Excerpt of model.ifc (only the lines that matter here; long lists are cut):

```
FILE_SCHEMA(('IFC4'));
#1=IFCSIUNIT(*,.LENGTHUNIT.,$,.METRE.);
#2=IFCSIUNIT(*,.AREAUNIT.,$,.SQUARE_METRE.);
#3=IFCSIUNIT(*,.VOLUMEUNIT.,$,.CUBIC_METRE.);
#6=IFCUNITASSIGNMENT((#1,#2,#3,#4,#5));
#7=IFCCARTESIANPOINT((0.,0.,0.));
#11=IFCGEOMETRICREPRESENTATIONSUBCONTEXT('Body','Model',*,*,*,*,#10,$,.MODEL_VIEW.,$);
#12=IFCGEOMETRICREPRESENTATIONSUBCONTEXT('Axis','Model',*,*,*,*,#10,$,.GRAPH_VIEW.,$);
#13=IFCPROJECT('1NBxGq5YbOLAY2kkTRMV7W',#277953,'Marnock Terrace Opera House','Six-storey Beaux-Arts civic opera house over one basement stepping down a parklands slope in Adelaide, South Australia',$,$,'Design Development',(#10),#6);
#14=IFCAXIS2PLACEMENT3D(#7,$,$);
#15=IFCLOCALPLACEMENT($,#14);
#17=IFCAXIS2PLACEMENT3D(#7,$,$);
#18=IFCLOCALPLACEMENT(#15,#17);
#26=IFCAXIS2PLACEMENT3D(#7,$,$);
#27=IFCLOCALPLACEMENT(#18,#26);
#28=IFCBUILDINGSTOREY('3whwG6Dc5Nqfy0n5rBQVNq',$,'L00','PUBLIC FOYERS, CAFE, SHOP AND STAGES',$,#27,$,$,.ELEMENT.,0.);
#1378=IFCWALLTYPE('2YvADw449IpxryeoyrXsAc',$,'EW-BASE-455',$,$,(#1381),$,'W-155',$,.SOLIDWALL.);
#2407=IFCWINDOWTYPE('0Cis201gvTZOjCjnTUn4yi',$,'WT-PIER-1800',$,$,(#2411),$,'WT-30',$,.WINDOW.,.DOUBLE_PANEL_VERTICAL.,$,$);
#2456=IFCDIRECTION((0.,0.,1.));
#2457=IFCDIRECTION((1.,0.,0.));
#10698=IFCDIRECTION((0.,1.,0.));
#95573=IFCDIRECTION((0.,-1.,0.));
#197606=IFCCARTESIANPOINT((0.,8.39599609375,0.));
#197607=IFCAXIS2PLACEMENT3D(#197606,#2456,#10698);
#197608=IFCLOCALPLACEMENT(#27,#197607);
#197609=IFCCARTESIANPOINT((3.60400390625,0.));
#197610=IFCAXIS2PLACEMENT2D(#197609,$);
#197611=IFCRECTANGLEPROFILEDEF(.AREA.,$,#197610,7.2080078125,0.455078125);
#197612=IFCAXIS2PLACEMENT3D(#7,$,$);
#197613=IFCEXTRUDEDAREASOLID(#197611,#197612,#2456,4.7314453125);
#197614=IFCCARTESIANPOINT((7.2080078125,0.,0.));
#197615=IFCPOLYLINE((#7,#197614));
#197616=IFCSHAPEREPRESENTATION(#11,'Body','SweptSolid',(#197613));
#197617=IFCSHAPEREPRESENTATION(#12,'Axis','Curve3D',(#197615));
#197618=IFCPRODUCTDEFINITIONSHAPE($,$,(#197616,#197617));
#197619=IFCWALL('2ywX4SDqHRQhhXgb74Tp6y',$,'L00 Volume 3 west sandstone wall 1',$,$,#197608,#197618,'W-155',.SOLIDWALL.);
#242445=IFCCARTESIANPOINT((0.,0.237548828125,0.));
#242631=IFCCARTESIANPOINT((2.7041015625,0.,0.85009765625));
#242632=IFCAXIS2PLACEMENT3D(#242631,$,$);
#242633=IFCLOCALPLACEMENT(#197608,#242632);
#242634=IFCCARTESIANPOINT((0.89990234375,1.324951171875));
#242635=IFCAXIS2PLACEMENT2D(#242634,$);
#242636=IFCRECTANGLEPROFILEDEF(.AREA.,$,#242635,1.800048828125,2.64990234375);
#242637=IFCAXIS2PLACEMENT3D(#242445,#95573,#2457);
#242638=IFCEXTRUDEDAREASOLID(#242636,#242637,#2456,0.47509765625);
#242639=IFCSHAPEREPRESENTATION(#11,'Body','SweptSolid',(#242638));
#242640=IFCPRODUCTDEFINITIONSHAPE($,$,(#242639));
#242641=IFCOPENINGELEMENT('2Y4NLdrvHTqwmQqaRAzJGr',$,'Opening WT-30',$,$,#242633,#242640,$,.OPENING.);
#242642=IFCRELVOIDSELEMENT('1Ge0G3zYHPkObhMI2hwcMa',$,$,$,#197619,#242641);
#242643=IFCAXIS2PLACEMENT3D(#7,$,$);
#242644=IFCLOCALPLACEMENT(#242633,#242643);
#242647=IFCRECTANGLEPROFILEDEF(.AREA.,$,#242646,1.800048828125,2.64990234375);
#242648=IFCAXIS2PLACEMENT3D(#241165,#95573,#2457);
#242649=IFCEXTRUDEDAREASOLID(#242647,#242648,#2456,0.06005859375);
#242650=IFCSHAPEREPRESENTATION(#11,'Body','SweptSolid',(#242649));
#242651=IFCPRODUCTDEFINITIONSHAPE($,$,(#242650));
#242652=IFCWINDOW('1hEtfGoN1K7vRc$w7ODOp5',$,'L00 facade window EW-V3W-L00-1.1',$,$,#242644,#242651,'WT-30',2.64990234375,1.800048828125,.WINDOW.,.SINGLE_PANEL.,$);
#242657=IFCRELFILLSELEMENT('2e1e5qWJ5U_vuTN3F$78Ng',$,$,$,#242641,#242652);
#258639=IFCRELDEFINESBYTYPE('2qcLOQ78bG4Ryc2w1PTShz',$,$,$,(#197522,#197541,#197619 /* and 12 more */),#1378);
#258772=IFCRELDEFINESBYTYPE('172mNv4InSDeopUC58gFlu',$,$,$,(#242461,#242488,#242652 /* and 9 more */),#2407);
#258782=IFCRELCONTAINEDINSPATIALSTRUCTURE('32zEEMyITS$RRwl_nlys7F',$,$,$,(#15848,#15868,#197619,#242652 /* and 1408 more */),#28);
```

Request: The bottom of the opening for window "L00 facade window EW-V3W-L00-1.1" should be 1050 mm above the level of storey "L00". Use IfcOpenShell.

```python
import numpy as np
import ifcopenshell
import ifcopenshell.api.geometry
import ifcopenshell.geom
import ifcopenshell.util.element
import ifcopenshell.util.placement
import ifcopenshell.util.shape
import ifcopenshell.util.unit

model = ifcopenshell.open("model.ifc")
unit_scale = ifcopenshell.util.unit.calculate_unit_scale(model)

window = model.by_guid("1hEtfGoN1K7vRc$w7ODOp5")
opening = window.FillsVoids[0].RelatingOpeningElement
storey = ifcopenshell.util.element.get_container(window, ifc_class="IfcBuildingStorey")
level = ifcopenshell.util.placement.get_local_placement(storey.ObjectPlacement)[2, 3]

# The opening's origin need not be at the sill, so measure its lowest point.
shape = ifcopenshell.geom.create_shape(ifcopenshell.geom.settings(), opening)
bottom = ifcopenshell.util.shape.get_shape_bottom_elevation(shape, shape.geometry) / unit_scale
dz = level + 1.05 - bottom

shift = np.array([0.0, 0.0, dz])
# The window is placed relative to its opening, so it follows when the opening moves.
matrix = ifcopenshell.util.placement.get_local_placement(opening.ObjectPlacement)
matrix[:3, 3] += shift
ifcopenshell.api.geometry.edit_object_placement(
    model, product=opening, matrix=matrix, is_si=False, should_transform_children=True
)

print(f"moved by {dz * unit_scale:+.3f} m")

model.write("model-out.ifc")
```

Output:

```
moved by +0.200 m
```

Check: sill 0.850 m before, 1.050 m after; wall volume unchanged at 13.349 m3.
